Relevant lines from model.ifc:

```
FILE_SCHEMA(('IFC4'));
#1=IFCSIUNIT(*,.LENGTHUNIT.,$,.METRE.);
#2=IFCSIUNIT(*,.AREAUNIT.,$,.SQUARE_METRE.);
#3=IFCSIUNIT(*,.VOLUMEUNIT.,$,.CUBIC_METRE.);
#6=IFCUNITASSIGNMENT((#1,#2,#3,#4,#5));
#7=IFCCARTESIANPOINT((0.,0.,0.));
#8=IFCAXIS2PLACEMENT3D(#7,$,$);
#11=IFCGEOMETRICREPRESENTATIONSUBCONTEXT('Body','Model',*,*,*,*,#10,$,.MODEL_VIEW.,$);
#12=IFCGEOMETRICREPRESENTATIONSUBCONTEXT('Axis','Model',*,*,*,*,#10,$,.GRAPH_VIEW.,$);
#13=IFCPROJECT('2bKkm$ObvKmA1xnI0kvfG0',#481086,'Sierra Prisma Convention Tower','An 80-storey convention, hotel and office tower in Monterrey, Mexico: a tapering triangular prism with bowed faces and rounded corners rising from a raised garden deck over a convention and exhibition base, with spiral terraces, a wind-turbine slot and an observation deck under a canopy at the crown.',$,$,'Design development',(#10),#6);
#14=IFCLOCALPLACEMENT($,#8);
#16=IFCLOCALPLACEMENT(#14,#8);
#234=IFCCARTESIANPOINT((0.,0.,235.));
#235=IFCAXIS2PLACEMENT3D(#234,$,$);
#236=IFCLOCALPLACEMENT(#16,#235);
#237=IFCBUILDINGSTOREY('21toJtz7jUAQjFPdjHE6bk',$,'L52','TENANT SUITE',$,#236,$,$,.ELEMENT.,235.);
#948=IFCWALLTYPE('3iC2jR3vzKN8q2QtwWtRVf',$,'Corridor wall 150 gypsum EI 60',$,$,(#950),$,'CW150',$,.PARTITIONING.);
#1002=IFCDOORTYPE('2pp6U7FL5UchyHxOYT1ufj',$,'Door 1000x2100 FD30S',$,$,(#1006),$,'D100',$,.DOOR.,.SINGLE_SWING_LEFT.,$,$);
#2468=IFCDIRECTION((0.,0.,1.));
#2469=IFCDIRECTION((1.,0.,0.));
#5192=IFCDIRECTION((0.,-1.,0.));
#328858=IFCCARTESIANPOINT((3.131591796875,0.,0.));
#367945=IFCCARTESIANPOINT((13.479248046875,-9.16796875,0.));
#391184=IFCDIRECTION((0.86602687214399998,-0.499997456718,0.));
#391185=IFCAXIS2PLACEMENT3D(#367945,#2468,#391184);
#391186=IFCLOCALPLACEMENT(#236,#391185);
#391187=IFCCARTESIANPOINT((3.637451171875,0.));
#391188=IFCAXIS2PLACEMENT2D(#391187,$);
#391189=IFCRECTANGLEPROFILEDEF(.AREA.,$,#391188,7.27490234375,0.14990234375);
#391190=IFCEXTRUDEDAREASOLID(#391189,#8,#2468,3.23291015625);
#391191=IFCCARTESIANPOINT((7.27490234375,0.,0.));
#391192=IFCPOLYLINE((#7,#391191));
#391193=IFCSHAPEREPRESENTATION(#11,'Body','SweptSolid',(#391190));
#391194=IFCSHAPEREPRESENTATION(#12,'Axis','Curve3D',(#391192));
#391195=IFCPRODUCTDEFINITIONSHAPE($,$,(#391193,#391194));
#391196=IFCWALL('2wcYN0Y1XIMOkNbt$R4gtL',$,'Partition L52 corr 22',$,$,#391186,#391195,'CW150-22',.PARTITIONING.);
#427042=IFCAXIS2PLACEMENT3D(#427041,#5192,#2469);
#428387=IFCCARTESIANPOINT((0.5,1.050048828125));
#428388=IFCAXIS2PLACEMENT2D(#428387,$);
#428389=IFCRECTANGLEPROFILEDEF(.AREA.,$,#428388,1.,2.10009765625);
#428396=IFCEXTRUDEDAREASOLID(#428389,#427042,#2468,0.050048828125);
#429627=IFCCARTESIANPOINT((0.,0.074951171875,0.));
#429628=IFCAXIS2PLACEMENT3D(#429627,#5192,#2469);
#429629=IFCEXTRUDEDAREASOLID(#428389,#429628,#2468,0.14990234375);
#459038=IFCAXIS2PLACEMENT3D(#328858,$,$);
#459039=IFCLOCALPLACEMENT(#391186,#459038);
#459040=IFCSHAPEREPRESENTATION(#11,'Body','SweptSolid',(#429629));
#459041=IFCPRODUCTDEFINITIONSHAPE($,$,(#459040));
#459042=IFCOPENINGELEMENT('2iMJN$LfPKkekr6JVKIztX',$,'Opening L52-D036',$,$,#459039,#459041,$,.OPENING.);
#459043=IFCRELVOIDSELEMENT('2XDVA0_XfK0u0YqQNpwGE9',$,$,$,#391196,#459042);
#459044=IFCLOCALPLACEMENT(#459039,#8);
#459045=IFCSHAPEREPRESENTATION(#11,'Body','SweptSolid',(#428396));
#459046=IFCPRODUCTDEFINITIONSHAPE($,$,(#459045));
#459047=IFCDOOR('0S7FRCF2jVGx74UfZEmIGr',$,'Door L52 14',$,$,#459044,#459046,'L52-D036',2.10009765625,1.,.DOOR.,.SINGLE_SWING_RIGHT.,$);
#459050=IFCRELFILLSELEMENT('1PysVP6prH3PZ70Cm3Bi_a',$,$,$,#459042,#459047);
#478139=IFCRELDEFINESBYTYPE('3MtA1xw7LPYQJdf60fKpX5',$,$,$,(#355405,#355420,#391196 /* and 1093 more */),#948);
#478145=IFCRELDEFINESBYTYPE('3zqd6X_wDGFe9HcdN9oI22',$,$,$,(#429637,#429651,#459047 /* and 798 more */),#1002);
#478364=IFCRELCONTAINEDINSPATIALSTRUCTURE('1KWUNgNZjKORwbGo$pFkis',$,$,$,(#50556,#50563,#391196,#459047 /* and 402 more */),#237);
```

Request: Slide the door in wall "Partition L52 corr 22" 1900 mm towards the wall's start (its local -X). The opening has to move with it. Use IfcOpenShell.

```python
import ifcopenshell
import ifcopenshell.api.geometry
import ifcopenshell.util.placement
import ifcopenshell.util.unit

model = ifcopenshell.open("model.ifc")
unit_scale = ifcopenshell.util.unit.calculate_unit_scale(model)

door = model.by_guid("0S7FRCF2jVGx74UfZEmIGr")
opening = door.FillsVoids[0].RelatingOpeningElement
wall = opening.VoidsElements[0].RelatingBuildingElement

wall_matrix = ifcopenshell.util.placement.get_local_placement(wall.ObjectPlacement)
shift = wall_matrix[:3, 0] * -1.9 / unit_scale
before = ifcopenshell.util.placement.get_local_placement(door.ObjectPlacement)[:3, 3].copy()

# The door is placed relative to its opening, so it follows when the opening moves.
matrix = ifcopenshell.util.placement.get_local_placement(opening.ObjectPlacement)
matrix[:3, 3] += shift
ifcopenshell.api.geometry.edit_object_placement(
    model, product=opening, matrix=matrix, is_si=False, should_transform_children=True
)

after = ifcopenshell.util.placement.get_local_placement(door.ObjectPlacement)[:3, 3]
print("door moved by", (after - before).round(3) + 0.0)

model.write("model-out.ifc")
```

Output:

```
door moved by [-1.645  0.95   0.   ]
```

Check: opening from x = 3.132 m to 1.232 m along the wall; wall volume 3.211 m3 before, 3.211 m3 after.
